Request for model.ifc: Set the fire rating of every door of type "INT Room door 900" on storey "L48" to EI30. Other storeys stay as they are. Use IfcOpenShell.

First a look at what the model holds.

```python
import ifcopenshell
import ifcopenshell.util.element

model = ifcopenshell.open("model.ifc")
print(model.schema)
storey = next(s for s in model.by_type("IfcBuildingStorey") if s.Name == "L48")
doors = [e for e in ifcopenshell.util.element.get_decomposition(storey) if e.is_a("IfcDoor")]
seen = {}
for e in doors:
    element_type = ifcopenshell.util.element.get_type(e)
    key = (element_type.Name if element_type != e and element_type else None, ifcopenshell.util.element.get_pset(e, "Pset_DoorCommon", "FireRating"))
    seen[key] = seen.get(key, 0) + 1
for (name, value), count in sorted(seen.items(), key=str):
    print(count, "x", name, "|", value)
```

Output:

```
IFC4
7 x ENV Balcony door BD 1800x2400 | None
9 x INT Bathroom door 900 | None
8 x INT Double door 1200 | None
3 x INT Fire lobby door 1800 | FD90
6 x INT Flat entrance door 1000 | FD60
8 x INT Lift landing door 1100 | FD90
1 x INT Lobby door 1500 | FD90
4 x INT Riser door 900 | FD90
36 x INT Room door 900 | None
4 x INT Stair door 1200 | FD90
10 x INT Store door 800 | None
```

```python
import ifcopenshell
import ifcopenshell.api.pset
import ifcopenshell.util.element

model = ifcopenshell.open("model.ifc")

storey = next(s for s in model.by_type("IfcBuildingStorey") if s.Name == "L48")
doors = [e for e in ifcopenshell.util.element.get_decomposition(storey) if e.is_a("IfcDoor")]

count = 0
for e in doors:
    element_type = ifcopenshell.util.element.get_type(e)
    if element_type in (None, e) or element_type.Name != "INT Room door 900":
        continue
    found = ifcopenshell.util.element.get_pset(e, "Pset_DoorCommon", should_inherit=False)
    if found:
        pset = model.by_id(found["id"])
        if len(ifcopenshell.util.element.get_elements_by_pset(pset)) > 1:
            pset = ifcopenshell.api.pset.unshare_pset(model, products=[e], pset=pset)[0]
    else:
        pset = ifcopenshell.api.pset.add_pset(model, product=e, name="Pset_DoorCommon")
    ifcopenshell.api.pset.edit_pset(model, pset=pset, properties={"FireRating": "EI30"})
    count += 1

print(count, "doors updated")

model.write("model-out.ifc")
```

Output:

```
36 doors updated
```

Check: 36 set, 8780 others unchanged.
